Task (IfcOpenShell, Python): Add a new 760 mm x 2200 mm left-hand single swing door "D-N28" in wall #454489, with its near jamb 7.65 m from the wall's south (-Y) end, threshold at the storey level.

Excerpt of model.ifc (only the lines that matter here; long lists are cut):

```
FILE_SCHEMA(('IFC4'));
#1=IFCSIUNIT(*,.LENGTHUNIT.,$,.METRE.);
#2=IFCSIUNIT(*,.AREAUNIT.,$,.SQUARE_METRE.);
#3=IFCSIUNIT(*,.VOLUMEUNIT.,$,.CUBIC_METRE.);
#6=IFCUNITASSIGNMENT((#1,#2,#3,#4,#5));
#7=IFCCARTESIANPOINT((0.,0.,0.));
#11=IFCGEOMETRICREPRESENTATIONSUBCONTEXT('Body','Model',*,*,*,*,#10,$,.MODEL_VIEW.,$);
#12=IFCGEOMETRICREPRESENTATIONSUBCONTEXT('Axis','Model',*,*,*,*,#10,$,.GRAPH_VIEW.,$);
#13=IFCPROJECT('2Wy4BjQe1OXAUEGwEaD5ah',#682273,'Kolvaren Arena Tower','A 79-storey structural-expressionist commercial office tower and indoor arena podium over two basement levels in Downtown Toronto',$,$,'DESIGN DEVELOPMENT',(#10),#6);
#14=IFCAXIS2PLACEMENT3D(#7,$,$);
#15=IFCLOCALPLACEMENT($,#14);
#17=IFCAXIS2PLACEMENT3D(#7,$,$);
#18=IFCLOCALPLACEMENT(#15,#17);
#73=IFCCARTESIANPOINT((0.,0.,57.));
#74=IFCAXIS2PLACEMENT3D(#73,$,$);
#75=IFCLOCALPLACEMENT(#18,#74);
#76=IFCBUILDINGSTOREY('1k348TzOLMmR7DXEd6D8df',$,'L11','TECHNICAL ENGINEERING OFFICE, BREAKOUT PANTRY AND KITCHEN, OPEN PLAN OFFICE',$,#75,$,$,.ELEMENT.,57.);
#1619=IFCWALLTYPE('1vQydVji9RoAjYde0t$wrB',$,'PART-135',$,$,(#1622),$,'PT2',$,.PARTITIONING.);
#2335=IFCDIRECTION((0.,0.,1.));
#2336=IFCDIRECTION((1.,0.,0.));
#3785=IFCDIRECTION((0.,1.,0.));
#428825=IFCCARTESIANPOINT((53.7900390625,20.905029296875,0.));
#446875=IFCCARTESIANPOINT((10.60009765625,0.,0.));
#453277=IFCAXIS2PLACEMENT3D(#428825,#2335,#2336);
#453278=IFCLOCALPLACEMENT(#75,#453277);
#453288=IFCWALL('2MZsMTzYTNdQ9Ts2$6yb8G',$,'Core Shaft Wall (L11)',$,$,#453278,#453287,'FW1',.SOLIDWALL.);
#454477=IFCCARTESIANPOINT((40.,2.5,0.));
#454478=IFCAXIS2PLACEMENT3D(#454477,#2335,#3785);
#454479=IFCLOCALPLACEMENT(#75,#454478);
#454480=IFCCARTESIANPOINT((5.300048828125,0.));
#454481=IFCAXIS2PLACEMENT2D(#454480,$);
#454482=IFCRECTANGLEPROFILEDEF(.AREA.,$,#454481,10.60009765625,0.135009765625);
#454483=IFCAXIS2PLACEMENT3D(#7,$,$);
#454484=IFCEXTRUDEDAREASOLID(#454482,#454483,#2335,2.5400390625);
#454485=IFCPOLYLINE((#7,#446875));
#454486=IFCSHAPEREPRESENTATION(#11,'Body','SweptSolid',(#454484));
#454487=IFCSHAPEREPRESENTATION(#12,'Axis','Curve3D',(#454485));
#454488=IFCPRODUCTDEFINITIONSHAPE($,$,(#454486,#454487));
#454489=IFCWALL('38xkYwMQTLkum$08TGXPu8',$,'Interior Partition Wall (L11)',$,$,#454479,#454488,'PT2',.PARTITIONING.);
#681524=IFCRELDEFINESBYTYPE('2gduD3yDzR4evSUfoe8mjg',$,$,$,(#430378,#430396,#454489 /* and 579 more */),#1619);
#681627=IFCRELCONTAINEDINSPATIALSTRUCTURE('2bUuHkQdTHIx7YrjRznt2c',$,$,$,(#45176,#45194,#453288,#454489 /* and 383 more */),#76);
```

```python
import numpy as np
import ifcopenshell
import ifcopenshell.api.feature
import ifcopenshell.api.geometry
import ifcopenshell.api.root
import ifcopenshell.api.spatial
import ifcopenshell.geom
import ifcopenshell.util.element
import ifcopenshell.util.placement
import ifcopenshell.util.representation
import ifcopenshell.util.shape
import ifcopenshell.util.unit

model = ifcopenshell.open("model.ifc")
unit_scale = ifcopenshell.util.unit.calculate_unit_scale(model)
settings = ifcopenshell.geom.settings()


def volume(element):
    """Net volume in cubic metres, openings subtracted."""
    shape = ifcopenshell.geom.create_shape(settings, element)
    return ifcopenshell.util.shape.get_volume(shape.geometry)


wall = model.by_guid("38xkYwMQTLkum$08TGXPu8")
storey = ifcopenshell.util.element.get_container(wall, ifc_class="IfcBuildingStorey")
context = ifcopenshell.util.representation.get_context(model, "Model", "Body", "MODEL_VIEW")
before = volume(wall)

width, height, from_end, sill = 0.76, 2.2, 7.65, 0.0  # metres

# The wall runs along its own X axis, and the end named is its -X end.
wall_shape = ifcopenshell.geom.create_shape(settings, wall)
x, y, z = ifcopenshell.util.shape.get_vertices(wall_shape.geometry).T
start = x.min() + from_end
face, thickness = float(y.min()), float(y.max() - y.min())
wall_matrix = ifcopenshell.util.placement.get_local_placement(wall.ObjectPlacement)
level = ifcopenshell.util.placement.get_local_placement(storey.ObjectPlacement)[2, 3]


def in_wall(x, y):
    """Placement at x, y metres in the wall's axes, at sill height."""
    matrix = wall_matrix.copy()
    matrix[:, 3] = wall_matrix @ np.array([x / unit_scale, y / unit_scale, 0.0, 1.0])
    matrix[2, 3] = level + sill / unit_scale
    return matrix


# Opening: a box that overshoots both wall faces by 50 mm.
opening = ifcopenshell.api.root.create_entity(model, ifc_class="IfcOpeningElement", predefined_type="OPENING")
box = ifcopenshell.api.geometry.add_wall_representation(
    model, context=context, length=width, height=height, thickness=thickness + 0.1
)
ifcopenshell.api.geometry.assign_representation(model, product=opening, representation=box)
ifcopenshell.api.geometry.edit_object_placement(model, product=opening, matrix=in_wall(start, face - 0.05), is_si=False)
ifcopenshell.api.feature.add_feature(model, feature=opening, element=wall)

door = ifcopenshell.api.root.create_entity(model, ifc_class="IfcDoor", name="D-N28", predefined_type="DOOR")
door.OverallWidth, door.OverallHeight = width / unit_scale, height / unit_scale
door.OperationType = "SINGLE_SWING_LEFT"
body = ifcopenshell.api.geometry.add_door_representation(
    model,
    context=context,
    overall_width=door.OverallWidth,
    overall_height=door.OverallHeight,
    operation_type="SINGLE_SWING_LEFT",
    lining_properties={"LiningDepth": thickness / unit_scale, "ThresholdDepth": thickness / unit_scale},
)
ifcopenshell.api.geometry.assign_representation(model, product=door, representation=body)
ifcopenshell.api.spatial.assign_container(model, products=[door], relating_structure=storey)
ifcopenshell.api.feature.add_filling(model, opening=opening, element=door)

# The lining spans the wall, so the door starts at the wall face.
ifcopenshell.api.geometry.edit_object_placement(model, product=door, matrix=in_wall(start, face), is_si=False)

after = volume(wall)

print(f"wall volume {before:.3f} -> {after:.3f} m3")

model.write("model_rev.ifc")
```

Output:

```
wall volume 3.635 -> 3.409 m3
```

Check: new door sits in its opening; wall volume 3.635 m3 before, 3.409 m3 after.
